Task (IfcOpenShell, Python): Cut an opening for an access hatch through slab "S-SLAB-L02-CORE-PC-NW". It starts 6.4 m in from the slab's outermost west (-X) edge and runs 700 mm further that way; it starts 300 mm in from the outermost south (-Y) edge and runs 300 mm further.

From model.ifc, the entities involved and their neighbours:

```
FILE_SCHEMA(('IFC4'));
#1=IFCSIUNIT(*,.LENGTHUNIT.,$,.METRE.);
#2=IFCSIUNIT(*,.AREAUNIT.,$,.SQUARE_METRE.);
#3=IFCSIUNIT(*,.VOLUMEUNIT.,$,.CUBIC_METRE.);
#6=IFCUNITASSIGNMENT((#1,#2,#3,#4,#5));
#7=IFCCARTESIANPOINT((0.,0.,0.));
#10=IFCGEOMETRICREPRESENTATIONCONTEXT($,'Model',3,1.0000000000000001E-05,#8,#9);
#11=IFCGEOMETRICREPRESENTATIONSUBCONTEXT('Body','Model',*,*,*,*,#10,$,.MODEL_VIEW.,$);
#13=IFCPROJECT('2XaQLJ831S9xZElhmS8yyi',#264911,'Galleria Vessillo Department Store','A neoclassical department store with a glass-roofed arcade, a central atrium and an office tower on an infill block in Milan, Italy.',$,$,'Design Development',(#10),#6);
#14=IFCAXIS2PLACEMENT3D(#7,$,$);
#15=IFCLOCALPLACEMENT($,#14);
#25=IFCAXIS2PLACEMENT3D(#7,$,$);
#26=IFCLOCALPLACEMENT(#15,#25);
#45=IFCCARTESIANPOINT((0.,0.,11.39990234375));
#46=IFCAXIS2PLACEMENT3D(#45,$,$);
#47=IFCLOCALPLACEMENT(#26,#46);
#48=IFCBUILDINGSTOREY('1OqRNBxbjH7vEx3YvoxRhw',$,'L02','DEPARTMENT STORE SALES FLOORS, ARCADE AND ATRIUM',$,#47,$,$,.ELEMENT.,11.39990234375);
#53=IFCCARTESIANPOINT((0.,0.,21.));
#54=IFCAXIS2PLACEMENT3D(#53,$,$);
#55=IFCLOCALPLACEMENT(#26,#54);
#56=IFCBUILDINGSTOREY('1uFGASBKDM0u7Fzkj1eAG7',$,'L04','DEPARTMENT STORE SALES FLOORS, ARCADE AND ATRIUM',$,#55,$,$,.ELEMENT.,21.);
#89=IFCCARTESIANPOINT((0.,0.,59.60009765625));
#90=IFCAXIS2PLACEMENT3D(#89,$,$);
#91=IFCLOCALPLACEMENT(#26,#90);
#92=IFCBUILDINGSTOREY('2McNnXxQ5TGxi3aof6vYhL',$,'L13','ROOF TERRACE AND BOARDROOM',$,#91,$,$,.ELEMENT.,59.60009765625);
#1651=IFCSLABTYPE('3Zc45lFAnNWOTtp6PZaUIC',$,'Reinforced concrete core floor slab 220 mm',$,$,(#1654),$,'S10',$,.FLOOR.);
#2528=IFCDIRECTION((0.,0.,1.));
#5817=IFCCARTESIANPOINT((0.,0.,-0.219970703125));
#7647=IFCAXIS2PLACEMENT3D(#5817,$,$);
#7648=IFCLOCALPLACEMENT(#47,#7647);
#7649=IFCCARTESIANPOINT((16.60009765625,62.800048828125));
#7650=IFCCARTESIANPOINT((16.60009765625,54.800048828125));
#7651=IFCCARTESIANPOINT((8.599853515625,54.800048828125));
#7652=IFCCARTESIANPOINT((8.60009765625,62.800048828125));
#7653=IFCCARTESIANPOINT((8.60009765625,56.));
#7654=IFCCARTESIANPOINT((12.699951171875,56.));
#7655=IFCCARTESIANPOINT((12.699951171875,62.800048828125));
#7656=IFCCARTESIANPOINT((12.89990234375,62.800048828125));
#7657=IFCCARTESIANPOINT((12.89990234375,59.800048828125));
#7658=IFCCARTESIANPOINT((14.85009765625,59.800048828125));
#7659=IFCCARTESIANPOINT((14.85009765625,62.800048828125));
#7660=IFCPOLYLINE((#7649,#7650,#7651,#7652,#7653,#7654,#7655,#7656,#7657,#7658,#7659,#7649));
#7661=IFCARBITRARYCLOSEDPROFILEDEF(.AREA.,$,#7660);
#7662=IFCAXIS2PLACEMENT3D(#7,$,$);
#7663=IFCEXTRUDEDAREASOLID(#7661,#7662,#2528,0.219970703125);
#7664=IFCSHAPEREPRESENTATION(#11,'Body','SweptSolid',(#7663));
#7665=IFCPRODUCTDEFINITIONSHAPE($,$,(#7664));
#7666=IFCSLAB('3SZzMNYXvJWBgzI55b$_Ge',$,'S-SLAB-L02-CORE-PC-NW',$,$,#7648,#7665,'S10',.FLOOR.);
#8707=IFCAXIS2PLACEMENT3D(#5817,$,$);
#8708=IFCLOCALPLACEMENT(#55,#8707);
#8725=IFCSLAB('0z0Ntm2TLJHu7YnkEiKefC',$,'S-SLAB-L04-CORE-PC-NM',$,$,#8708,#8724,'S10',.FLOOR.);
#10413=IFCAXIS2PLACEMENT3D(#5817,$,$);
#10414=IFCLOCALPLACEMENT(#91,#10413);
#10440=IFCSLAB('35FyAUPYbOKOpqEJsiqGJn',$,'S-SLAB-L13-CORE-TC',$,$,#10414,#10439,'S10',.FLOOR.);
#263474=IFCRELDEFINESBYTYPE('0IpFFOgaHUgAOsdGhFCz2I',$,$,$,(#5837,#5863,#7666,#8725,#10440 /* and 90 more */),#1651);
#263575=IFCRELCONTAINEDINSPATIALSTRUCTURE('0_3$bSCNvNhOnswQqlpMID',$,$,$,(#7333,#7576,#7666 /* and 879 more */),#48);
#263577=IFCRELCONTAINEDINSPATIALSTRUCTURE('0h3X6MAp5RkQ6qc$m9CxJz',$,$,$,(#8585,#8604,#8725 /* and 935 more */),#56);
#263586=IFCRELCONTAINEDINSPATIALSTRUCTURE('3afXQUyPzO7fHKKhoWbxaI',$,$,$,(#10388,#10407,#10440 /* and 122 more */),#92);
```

```python
import numpy as np
import ifcopenshell
import ifcopenshell.api.feature
import ifcopenshell.api.geometry
import ifcopenshell.api.root
import ifcopenshell.geom
import ifcopenshell.util.placement
import ifcopenshell.util.representation
import ifcopenshell.util.shape
import ifcopenshell.util.unit

model = ifcopenshell.open("model.ifc")
unit_scale = ifcopenshell.util.unit.calculate_unit_scale(model)
settings = ifcopenshell.geom.settings()


def volume(element):
    """Net volume in cubic metres, openings subtracted."""
    shape = ifcopenshell.geom.create_shape(settings, element)
    return ifcopenshell.util.shape.get_volume(shape.geometry)


slab = model.by_id(7666)
before = volume(slab)

# Extent in the slab's own axes, in metres. The edges named are its -X and -Y sides.
slab_shape = ifcopenshell.geom.create_shape(settings, slab)
vertices = ifcopenshell.util.shape.get_vertices(slab_shape.geometry)
x_min, y_min, bottom = vertices.min(axis=0)
top = vertices[:, 2].max()

opening = ifcopenshell.api.root.create_entity(model, ifc_class="IfcOpeningElement", name="Access hatch opening", predefined_type="OPENING")
context = ifcopenshell.util.representation.get_context(model, "Model", "Body", "MODEL_VIEW")
width, depth = 0.7, 0.3
outline = [(0.0, 0.0), (width, 0.0), (width, depth), (0.0, depth), (0.0, 0.0)]
# Overshoot both faces by 50 mm so the cut is clean.
shape = ifcopenshell.api.geometry.add_slab_representation(
    model, context=context, depth=top - bottom + 0.1, polyline=outline
)
ifcopenshell.api.geometry.assign_representation(model, product=opening, representation=shape)

matrix = ifcopenshell.util.placement.get_local_placement(slab.ObjectPlacement)
matrix[:, 3] = matrix @ np.append(np.array([x_min + 6.4, y_min + 0.3, bottom - 0.05]) / unit_scale, 1.0)
ifcopenshell.api.geometry.edit_object_placement(model, product=opening, matrix=matrix, is_si=False)
ifcopenshell.api.feature.add_feature(model, feature=opening, element=slab)

after = volume(slab)

print(f"slab volume {before:.3f} -> {after:.3f} m3")

model.write("model_rev.ifc")
```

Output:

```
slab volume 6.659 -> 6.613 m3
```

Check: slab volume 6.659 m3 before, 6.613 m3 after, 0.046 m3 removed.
